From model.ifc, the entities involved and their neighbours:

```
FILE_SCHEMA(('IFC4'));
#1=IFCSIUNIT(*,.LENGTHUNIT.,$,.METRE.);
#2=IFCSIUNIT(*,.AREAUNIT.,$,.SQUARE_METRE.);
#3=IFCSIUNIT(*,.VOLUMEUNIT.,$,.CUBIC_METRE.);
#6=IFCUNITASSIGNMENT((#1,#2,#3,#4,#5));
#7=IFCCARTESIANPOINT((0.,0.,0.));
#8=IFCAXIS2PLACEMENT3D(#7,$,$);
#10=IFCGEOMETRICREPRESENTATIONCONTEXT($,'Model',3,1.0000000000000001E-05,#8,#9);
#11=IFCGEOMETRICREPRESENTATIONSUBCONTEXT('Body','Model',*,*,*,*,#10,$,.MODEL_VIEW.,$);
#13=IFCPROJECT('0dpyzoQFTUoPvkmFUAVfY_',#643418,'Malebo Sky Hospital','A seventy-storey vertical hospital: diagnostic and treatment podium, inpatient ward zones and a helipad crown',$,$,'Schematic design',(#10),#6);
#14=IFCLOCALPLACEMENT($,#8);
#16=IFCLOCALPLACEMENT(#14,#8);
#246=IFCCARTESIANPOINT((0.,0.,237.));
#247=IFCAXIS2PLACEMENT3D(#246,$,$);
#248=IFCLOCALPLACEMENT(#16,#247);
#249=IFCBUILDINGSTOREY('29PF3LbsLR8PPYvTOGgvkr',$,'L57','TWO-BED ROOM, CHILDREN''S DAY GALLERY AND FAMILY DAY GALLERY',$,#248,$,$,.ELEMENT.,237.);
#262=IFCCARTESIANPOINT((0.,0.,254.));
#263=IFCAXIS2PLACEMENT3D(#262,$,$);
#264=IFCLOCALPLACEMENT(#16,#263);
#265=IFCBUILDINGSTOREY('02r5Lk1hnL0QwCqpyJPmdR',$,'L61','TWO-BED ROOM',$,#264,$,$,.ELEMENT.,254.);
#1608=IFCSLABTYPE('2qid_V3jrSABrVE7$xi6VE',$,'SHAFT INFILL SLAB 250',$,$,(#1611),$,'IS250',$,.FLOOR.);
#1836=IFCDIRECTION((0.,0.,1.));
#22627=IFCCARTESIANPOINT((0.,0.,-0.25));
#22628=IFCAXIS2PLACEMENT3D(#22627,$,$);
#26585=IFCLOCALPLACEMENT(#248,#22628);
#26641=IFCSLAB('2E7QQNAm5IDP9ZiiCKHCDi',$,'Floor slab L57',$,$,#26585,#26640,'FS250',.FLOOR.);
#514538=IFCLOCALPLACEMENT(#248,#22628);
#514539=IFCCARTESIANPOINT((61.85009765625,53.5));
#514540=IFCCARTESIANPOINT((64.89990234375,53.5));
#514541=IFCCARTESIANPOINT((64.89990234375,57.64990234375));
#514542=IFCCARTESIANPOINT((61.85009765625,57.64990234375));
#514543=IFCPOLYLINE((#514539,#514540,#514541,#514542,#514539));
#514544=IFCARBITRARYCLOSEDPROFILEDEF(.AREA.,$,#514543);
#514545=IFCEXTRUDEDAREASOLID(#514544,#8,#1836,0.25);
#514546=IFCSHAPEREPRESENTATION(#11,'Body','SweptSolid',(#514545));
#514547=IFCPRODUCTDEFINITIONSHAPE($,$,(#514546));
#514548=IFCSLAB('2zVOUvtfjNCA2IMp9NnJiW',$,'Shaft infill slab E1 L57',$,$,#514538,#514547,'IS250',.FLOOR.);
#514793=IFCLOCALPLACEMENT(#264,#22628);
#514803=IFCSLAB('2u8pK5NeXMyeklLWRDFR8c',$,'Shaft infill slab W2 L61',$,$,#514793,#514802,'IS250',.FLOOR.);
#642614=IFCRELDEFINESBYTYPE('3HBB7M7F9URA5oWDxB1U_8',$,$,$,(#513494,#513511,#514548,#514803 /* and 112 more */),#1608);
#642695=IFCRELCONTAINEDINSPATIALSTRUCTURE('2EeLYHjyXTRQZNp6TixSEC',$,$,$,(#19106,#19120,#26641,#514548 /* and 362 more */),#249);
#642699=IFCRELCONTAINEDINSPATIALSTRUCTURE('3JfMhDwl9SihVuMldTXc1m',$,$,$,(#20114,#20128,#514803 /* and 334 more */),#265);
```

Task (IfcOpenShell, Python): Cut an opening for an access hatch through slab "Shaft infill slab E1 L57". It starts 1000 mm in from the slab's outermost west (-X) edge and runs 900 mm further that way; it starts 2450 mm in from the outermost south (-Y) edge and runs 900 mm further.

```python
import numpy as np
import ifcopenshell
import ifcopenshell.api.feature
import ifcopenshell.api.geometry
import ifcopenshell.api.root
import ifcopenshell.geom
import ifcopenshell.util.placement
import ifcopenshell.util.representation
import ifcopenshell.util.shape
import ifcopenshell.util.unit

model = ifcopenshell.open("model.ifc")
unit_scale = ifcopenshell.util.unit.calculate_unit_scale(model)
settings = ifcopenshell.geom.settings()


def volume(element):
    """Net volume in cubic metres, openings subtracted."""
    shape = ifcopenshell.geom.create_shape(settings, element)
    return ifcopenshell.util.shape.get_volume(shape.geometry)


slab = model.by_guid("2zVOUvtfjNCA2IMp9NnJiW")
before = volume(slab)

# Extent in the slab's own axes, in metres. The edges named are its -X and -Y sides.
slab_shape = ifcopenshell.geom.create_shape(settings, slab)
vertices = ifcopenshell.util.shape.get_vertices(slab_shape.geometry)
x_min, y_min, bottom = vertices.min(axis=0)
top = vertices[:, 2].max()

opening = ifcopenshell.api.root.create_entity(model, ifc_class="IfcOpeningElement", name="Access hatch opening", predefined_type="OPENING")
context = ifcopenshell.util.representation.get_context(model, "Model", "Body", "MODEL_VIEW")
width, depth = 0.9, 0.9
outline = [(0.0, 0.0), (width, 0.0), (width, depth), (0.0, depth), (0.0, 0.0)]
# Overshoot both faces by 50 mm so the cut is clean.
shape = ifcopenshell.api.geometry.add_slab_representation(
    model, context=context, depth=top - bottom + 0.1, polyline=outline
)
ifcopenshell.api.geometry.assign_representation(model, product=opening, representation=shape)

matrix = ifcopenshell.util.placement.get_local_placement(slab.ObjectPlacement)
matrix[:, 3] = matrix @ np.append(np.array([x_min + 1, y_min + 2.45, bottom - 0.05]) / unit_scale, 1.0)
ifcopenshell.api.geometry.edit_object_placement(model, product=opening, matrix=matrix, is_si=False)
ifcopenshell.api.feature.add_feature(model, feature=opening, element=slab)

after = volume(slab)

print(f"slab volume {before:.3f} -> {after:.3f} m3")

model.write("model_rev.ifc")
```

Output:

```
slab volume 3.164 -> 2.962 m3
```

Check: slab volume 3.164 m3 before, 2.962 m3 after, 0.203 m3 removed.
